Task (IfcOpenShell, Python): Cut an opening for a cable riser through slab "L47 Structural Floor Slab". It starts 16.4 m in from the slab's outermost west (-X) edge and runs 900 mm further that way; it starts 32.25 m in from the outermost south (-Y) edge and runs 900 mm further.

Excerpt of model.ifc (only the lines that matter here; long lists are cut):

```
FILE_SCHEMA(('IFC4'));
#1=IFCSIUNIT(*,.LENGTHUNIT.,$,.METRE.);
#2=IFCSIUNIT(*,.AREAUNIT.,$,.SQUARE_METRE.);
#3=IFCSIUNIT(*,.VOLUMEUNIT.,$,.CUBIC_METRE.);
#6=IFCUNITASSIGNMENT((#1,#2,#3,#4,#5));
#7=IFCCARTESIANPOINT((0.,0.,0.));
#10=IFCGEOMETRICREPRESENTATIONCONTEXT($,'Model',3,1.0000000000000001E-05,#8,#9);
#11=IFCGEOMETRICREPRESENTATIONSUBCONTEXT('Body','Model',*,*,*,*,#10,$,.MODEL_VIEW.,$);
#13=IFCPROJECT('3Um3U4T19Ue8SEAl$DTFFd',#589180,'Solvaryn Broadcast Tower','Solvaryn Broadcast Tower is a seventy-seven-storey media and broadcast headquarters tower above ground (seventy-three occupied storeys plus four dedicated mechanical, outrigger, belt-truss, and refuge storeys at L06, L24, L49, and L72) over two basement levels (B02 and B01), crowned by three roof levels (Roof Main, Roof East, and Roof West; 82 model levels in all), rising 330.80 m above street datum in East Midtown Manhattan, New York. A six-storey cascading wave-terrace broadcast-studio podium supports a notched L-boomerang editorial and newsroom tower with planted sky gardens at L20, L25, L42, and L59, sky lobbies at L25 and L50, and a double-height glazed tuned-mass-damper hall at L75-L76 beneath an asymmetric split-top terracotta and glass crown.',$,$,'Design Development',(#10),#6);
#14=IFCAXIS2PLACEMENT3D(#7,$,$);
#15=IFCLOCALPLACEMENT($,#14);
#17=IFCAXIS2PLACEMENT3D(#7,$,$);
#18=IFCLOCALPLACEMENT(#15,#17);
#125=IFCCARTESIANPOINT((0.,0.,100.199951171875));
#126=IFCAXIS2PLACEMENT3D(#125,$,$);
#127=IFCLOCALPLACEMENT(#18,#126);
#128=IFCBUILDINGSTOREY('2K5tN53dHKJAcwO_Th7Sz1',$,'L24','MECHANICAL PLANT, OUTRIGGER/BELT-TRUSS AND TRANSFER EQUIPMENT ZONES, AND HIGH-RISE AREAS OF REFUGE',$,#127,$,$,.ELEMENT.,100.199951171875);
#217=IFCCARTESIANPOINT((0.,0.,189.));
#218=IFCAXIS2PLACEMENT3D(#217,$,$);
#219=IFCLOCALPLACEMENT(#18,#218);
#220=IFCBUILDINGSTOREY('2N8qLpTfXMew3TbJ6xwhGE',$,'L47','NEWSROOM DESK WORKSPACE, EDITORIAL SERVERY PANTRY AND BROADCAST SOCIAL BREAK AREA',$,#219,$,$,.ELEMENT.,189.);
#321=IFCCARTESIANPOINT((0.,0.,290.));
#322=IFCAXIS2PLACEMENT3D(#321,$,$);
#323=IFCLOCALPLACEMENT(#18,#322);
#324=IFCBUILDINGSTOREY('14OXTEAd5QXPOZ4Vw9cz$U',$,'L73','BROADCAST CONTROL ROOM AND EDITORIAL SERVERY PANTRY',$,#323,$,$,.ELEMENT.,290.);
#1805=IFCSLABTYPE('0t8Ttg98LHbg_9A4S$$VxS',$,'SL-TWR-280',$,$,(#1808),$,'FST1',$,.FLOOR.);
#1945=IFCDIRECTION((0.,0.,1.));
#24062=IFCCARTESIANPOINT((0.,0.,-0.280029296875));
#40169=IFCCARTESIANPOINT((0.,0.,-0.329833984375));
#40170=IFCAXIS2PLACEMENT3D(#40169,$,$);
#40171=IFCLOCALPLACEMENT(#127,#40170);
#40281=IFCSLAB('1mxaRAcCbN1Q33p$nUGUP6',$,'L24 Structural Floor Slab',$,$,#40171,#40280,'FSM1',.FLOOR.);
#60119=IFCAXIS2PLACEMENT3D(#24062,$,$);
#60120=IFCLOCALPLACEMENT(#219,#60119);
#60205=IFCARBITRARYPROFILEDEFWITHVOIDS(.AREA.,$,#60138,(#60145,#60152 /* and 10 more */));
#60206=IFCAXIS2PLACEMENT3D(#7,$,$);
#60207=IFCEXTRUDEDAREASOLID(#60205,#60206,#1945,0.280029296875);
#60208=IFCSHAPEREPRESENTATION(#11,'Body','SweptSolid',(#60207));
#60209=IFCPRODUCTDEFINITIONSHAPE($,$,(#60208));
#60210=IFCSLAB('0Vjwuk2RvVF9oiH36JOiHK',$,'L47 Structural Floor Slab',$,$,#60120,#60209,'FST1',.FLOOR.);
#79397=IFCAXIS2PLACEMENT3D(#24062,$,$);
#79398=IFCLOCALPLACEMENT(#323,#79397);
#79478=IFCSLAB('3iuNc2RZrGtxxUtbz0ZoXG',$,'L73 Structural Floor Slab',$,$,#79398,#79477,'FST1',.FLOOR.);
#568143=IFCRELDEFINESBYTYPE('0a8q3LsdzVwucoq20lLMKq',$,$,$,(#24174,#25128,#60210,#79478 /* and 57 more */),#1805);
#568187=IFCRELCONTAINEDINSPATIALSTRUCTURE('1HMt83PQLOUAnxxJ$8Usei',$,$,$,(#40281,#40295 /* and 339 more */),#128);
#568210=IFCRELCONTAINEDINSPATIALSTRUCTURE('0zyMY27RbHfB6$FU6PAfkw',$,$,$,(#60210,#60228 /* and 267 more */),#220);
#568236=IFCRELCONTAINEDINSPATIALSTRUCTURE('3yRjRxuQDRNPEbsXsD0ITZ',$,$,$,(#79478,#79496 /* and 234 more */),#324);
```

```python
import numpy as np
import ifcopenshell
import ifcopenshell.api.feature
import ifcopenshell.api.geometry
import ifcopenshell.api.root
import ifcopenshell.geom
import ifcopenshell.util.placement
import ifcopenshell.util.representation
import ifcopenshell.util.shape
import ifcopenshell.util.unit

model = ifcopenshell.open("model.ifc")
unit_scale = ifcopenshell.util.unit.calculate_unit_scale(model)
settings = ifcopenshell.geom.settings()


def volume(element):
    """Net volume in cubic metres, openings subtracted."""
    shape = ifcopenshell.geom.create_shape(settings, element)
    return ifcopenshell.util.shape.get_volume(shape.geometry)


slab = model.by_guid("0Vjwuk2RvVF9oiH36JOiHK")
before = volume(slab)

# Extent in the slab's own axes, in metres. The edges named are its -X and -Y sides.
slab_shape = ifcopenshell.geom.create_shape(settings, slab)
vertices = ifcopenshell.util.shape.get_vertices(slab_shape.geometry)
x_min, y_min, bottom = vertices.min(axis=0)
top = vertices[:, 2].max()

opening = ifcopenshell.api.root.create_entity(model, ifc_class="IfcOpeningElement", name="Cable riser opening", predefined_type="OPENING")
context = ifcopenshell.util.representation.get_context(model, "Model", "Body", "MODEL_VIEW")
width, depth = 0.9, 0.9
outline = [(0.0, 0.0), (width, 0.0), (width, depth), (0.0, depth), (0.0, 0.0)]
# Overshoot both faces by 50 mm so the cut is clean.
shape = ifcopenshell.api.geometry.add_slab_representation(
    model, context=context, depth=top - bottom + 0.1, polyline=outline
)
ifcopenshell.api.geometry.assign_representation(model, product=opening, representation=shape)

matrix = ifcopenshell.util.placement.get_local_placement(slab.ObjectPlacement)
matrix[:, 3] = matrix @ np.append(np.array([x_min + 16.4, y_min + 32.25, bottom - 0.05]) / unit_scale, 1.0)
ifcopenshell.api.geometry.edit_object_placement(model, product=opening, matrix=matrix, is_si=False)
ifcopenshell.api.feature.add_feature(model, feature=opening, element=slab)

after = volume(slab)

print(f"slab volume {before:.3f} -> {after:.3f} m3")

model.write("model-out.ifc")
```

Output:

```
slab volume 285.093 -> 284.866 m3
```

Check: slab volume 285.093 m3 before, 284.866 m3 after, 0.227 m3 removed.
